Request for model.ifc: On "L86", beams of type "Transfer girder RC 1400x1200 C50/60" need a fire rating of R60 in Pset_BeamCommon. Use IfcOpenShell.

First a look at what the model holds.

```python
import ifcopenshell
import ifcopenshell.util.element

model = ifcopenshell.open("model.ifc")
print(model.schema)
storey = next(s for s in model.by_type("IfcBuildingStorey") if s.Name == "L86")
beams = [e for e in ifcopenshell.util.element.get_decomposition(storey) if e.is_a("IfcBeam")]
seen = {}
for e in beams:
    element_type = ifcopenshell.util.element.get_type(e)
    key = (element_type.Name if element_type != e and element_type else None, ifcopenshell.util.element.get_pset(e, "Pset_BeamCommon", "FireRating"))
    seen[key] = seen.get(key, 0) + 1
for (name, value), count in sorted(seen.items(), key=str):
    print(count, "x", name, "|", value)
```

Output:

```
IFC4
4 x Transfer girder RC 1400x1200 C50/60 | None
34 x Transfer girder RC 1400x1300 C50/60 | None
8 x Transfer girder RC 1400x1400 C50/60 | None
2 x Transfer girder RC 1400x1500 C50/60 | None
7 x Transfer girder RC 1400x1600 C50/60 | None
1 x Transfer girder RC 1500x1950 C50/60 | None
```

```python
import ifcopenshell
import ifcopenshell.api.pset
import ifcopenshell.util.element

model = ifcopenshell.open("model.ifc")

storey = next(s for s in model.by_type("IfcBuildingStorey") if s.Name == "L86")
beams = [e for e in ifcopenshell.util.element.get_decomposition(storey) if e.is_a("IfcBeam")]

count = 0
for e in beams:
    element_type = ifcopenshell.util.element.get_type(e)
    if element_type in (None, e) or element_type.Name != "Transfer girder RC 1400x1200 C50/60":
        continue
    found = ifcopenshell.util.element.get_pset(e, "Pset_BeamCommon", should_inherit=False)
    if found:
        pset = model.by_id(found["id"])
        if len(ifcopenshell.util.element.get_elements_by_pset(pset)) > 1:
            pset = ifcopenshell.api.pset.unshare_pset(model, products=[e], pset=pset)[0]
    else:
        pset = ifcopenshell.api.pset.add_pset(model, product=e, name="Pset_BeamCommon")
    ifcopenshell.api.pset.edit_pset(model, pset=pset, properties={"FireRating": "R60"})
    count += 1

print(count, "beams updated")

model.write("model_edited.ifc")
```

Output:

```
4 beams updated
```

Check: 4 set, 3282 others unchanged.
